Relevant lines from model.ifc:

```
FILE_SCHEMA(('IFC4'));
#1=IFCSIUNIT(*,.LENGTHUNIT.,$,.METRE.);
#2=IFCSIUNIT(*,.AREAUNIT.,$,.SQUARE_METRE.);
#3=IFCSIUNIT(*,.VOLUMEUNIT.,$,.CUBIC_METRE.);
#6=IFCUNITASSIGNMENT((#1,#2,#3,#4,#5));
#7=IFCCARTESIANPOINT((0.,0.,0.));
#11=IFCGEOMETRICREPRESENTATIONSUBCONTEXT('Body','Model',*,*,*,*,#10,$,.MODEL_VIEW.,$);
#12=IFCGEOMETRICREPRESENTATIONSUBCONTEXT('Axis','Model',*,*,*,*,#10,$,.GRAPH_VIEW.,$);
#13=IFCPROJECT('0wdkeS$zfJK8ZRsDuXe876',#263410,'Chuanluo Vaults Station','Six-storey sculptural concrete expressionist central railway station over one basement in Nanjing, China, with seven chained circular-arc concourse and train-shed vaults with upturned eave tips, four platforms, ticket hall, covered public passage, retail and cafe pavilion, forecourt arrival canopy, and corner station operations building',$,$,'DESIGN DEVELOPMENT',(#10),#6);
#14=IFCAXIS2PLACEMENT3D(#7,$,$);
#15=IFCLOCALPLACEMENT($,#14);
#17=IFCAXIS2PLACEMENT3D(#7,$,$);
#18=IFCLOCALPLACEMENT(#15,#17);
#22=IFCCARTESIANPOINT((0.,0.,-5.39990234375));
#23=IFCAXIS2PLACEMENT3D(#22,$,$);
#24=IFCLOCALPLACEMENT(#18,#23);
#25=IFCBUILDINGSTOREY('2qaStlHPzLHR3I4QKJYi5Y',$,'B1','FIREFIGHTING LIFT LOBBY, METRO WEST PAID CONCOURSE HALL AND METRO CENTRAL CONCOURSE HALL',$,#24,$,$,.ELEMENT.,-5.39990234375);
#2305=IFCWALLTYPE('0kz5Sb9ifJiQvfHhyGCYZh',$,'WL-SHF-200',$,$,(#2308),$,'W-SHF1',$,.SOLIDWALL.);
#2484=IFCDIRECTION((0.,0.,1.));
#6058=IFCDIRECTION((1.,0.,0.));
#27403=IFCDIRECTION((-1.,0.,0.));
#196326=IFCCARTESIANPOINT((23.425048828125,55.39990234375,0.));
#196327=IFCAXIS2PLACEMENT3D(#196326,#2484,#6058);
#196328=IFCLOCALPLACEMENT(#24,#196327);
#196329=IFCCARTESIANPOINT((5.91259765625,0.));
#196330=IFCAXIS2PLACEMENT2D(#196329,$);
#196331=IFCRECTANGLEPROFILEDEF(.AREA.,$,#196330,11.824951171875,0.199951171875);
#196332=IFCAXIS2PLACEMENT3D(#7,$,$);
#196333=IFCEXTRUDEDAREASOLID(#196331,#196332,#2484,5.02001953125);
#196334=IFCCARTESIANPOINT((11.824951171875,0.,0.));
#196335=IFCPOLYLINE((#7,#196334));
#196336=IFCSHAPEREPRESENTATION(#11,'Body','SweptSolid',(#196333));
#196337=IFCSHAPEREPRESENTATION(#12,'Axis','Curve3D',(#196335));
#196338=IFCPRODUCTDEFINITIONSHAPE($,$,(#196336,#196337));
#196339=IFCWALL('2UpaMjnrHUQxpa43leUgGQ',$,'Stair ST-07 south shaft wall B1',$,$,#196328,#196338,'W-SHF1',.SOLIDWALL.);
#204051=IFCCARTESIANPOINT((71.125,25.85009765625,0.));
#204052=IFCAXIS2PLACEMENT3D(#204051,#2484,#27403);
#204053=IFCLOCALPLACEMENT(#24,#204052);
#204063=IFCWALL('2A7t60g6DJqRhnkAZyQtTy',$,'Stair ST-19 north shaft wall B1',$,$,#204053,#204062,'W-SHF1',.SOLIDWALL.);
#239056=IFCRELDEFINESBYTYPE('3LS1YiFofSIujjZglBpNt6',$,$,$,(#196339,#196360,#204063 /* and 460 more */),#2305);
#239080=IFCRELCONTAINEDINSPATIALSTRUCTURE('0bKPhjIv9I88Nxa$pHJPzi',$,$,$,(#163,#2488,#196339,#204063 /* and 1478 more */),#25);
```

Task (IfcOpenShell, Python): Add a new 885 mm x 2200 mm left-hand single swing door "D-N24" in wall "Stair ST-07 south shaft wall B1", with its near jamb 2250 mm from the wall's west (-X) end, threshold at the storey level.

```python
import numpy as np
import ifcopenshell
import ifcopenshell.api.feature
import ifcopenshell.api.geometry
import ifcopenshell.api.root
import ifcopenshell.api.spatial
import ifcopenshell.geom
import ifcopenshell.util.element
import ifcopenshell.util.placement
import ifcopenshell.util.representation
import ifcopenshell.util.shape
import ifcopenshell.util.unit

model = ifcopenshell.open("model.ifc")
unit_scale = ifcopenshell.util.unit.calculate_unit_scale(model)
settings = ifcopenshell.geom.settings()


def volume(element):
    """Net volume in cubic metres, openings subtracted."""
    shape = ifcopenshell.geom.create_shape(settings, element)
    return ifcopenshell.util.shape.get_volume(shape.geometry)


wall = model.by_id(196339)
storey = ifcopenshell.util.element.get_container(wall, ifc_class="IfcBuildingStorey")
context = ifcopenshell.util.representation.get_context(model, "Model", "Body", "MODEL_VIEW")
before = volume(wall)

width, height, from_end, sill = 0.885, 2.2, 2.25, 0.0  # metres

# The wall runs along its own X axis, and the end named is its -X end.
wall_shape = ifcopenshell.geom.create_shape(settings, wall)
x, y, z = ifcopenshell.util.shape.get_vertices(wall_shape.geometry).T
start = x.min() + from_end
face, thickness = float(y.min()), float(y.max() - y.min())
wall_matrix = ifcopenshell.util.placement.get_local_placement(wall.ObjectPlacement)
level = ifcopenshell.util.placement.get_local_placement(storey.ObjectPlacement)[2, 3]


def in_wall(x, y):
    """Placement at x, y metres in the wall's axes, at sill height."""
    matrix = wall_matrix.copy()
    matrix[:, 3] = wall_matrix @ np.array([x / unit_scale, y / unit_scale, 0.0, 1.0])
    matrix[2, 3] = level + sill / unit_scale
    return matrix


# Opening: a box that overshoots both wall faces by 50 mm.
opening = ifcopenshell.api.root.create_entity(model, ifc_class="IfcOpeningElement", predefined_type="OPENING")
box = ifcopenshell.api.geometry.add_wall_representation(
    model, context=context, length=width, height=height, thickness=thickness + 0.1
)
ifcopenshell.api.geometry.assign_representation(model, product=opening, representation=box)
ifcopenshell.api.geometry.edit_object_placement(model, product=opening, matrix=in_wall(start, face - 0.05), is_si=False)
ifcopenshell.api.feature.add_feature(model, feature=opening, element=wall)

door = ifcopenshell.api.root.create_entity(model, ifc_class="IfcDoor", name="D-N24", predefined_type="DOOR")
door.OverallWidth, door.OverallHeight = width / unit_scale, height / unit_scale
door.OperationType = "SINGLE_SWING_LEFT"
body = ifcopenshell.api.geometry.add_door_representation(
    model,
    context=context,
    overall_width=door.OverallWidth,
    overall_height=door.OverallHeight,
    operation_type="SINGLE_SWING_LEFT",
    lining_properties={"LiningDepth": thickness / unit_scale, "ThresholdDepth": thickness / unit_scale},
)
ifcopenshell.api.geometry.assign_representation(model, product=door, representation=body)
ifcopenshell.api.spatial.assign_container(model, products=[door], relating_structure=storey)
ifcopenshell.api.feature.add_filling(model, opening=opening, element=door)

# The lining spans the wall, so the door starts at the wall face.
ifcopenshell.api.geometry.edit_object_placement(model, product=door, matrix=in_wall(start, face), is_si=False)

after = volume(wall)

print(f"wall volume {before:.3f} -> {after:.3f} m3")

model.write("model_updated.ifc")
```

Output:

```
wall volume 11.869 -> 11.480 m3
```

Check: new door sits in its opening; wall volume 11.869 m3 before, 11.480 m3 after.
